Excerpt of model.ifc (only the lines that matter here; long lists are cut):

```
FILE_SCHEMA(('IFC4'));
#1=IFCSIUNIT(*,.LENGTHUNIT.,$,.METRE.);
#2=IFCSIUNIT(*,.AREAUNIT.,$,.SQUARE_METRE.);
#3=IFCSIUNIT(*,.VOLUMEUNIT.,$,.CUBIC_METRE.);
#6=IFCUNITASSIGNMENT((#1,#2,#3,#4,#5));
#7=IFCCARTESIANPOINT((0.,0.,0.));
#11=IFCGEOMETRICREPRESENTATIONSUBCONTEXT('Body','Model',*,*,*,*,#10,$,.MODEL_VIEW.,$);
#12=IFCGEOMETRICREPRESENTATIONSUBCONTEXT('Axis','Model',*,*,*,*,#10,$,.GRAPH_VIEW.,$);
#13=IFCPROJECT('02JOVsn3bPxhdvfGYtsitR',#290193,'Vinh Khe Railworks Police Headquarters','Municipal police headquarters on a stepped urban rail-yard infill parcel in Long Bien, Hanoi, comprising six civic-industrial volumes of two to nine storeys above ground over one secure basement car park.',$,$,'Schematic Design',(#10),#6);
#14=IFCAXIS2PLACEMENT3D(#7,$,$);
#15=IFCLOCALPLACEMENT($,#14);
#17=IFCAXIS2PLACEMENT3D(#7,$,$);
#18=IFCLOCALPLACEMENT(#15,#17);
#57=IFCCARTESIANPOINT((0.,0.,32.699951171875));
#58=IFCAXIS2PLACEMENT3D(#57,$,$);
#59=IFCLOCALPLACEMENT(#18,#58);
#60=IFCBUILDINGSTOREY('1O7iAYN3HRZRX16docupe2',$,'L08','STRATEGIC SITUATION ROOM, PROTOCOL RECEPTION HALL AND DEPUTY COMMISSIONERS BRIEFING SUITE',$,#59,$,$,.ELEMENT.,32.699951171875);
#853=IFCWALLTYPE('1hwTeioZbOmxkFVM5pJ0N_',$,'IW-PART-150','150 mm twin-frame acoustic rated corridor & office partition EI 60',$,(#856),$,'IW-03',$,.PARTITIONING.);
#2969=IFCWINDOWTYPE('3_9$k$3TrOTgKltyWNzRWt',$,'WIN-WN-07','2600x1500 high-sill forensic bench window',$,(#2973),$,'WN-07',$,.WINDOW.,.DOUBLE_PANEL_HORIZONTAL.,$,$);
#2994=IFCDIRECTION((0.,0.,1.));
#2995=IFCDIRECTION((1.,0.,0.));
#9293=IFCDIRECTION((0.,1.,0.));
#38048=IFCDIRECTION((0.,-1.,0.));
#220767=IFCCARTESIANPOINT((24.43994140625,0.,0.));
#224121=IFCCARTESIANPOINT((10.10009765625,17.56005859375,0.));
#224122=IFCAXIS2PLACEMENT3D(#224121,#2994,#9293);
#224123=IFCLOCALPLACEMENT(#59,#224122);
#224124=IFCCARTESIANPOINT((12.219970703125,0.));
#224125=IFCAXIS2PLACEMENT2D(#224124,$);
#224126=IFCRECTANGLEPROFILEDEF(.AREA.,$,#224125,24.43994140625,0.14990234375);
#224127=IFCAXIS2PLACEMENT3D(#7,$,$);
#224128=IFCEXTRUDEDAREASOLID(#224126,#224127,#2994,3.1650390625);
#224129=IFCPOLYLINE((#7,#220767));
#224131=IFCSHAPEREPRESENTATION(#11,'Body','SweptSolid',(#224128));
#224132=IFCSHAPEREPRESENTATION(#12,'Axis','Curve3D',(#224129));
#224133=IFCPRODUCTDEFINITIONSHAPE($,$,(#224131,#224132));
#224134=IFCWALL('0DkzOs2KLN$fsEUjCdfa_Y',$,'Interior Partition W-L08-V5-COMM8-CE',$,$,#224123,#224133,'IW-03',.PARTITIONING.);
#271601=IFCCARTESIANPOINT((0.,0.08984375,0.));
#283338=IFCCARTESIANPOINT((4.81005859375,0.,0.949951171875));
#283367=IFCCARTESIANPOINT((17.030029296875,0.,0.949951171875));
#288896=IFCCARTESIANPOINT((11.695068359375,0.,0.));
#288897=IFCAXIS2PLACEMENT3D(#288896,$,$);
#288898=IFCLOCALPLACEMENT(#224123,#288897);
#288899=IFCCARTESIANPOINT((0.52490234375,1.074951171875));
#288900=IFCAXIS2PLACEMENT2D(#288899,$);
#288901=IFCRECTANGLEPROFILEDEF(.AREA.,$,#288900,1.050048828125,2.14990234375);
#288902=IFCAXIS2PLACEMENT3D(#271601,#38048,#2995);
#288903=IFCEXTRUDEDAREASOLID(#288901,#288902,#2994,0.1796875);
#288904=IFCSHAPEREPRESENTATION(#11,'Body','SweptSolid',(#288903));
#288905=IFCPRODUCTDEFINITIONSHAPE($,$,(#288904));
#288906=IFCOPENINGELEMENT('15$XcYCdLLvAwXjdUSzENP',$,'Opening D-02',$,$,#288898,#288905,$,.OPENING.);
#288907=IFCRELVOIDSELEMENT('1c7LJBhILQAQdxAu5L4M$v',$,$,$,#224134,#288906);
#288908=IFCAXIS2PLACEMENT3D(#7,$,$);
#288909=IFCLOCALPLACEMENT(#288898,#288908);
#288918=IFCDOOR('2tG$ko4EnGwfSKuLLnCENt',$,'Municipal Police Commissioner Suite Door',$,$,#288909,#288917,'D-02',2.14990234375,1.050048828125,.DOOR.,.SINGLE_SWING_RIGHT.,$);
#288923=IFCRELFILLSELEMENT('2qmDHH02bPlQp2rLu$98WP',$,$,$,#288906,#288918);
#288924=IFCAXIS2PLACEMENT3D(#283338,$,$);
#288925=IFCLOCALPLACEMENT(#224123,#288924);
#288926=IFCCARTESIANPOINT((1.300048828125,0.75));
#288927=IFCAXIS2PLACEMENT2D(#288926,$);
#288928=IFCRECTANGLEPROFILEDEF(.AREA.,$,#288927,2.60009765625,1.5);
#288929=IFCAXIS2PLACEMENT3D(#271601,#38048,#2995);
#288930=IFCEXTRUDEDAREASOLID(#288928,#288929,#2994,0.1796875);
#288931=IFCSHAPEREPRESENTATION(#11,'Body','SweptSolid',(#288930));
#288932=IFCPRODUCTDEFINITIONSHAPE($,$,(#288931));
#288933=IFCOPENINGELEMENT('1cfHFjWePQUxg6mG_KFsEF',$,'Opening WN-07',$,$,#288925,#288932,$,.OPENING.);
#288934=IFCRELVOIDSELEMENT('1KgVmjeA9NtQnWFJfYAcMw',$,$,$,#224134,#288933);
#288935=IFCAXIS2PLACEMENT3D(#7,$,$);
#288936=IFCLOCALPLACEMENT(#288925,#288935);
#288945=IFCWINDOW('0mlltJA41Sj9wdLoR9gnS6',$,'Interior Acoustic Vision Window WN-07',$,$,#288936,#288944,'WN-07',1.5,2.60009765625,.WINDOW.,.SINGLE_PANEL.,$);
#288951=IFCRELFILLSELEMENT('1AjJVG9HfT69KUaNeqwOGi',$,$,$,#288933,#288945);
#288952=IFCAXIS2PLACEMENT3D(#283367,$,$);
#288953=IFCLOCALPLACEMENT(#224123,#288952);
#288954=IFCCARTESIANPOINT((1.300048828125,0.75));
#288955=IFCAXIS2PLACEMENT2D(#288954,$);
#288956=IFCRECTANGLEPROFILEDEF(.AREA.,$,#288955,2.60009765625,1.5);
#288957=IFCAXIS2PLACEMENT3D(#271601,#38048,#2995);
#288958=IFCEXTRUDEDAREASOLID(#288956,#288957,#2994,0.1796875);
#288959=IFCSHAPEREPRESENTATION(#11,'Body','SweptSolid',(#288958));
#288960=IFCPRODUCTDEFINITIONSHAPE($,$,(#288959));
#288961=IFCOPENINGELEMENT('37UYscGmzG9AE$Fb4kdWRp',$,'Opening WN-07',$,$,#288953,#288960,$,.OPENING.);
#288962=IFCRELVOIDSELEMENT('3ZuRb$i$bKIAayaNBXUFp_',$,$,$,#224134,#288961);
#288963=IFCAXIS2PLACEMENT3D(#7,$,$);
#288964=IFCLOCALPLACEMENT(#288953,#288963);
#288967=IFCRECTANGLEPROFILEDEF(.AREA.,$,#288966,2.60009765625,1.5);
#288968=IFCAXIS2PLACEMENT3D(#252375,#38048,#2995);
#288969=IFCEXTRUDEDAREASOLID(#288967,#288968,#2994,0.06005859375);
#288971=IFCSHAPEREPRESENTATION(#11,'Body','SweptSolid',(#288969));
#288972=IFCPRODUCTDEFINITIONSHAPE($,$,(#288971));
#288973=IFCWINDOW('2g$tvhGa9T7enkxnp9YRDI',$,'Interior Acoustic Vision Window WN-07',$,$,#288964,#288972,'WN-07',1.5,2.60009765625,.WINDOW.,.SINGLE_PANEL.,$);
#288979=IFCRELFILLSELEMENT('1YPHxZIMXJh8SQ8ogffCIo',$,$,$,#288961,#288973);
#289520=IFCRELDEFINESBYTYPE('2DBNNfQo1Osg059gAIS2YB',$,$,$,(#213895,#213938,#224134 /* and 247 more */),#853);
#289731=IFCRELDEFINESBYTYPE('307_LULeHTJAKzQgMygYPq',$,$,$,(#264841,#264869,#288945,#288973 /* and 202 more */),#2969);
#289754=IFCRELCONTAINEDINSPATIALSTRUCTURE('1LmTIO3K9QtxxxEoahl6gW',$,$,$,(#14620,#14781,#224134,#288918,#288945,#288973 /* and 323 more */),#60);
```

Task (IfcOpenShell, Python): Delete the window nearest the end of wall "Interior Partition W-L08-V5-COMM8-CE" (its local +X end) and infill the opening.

```python
import ifcopenshell
import ifcopenshell.api.feature
import ifcopenshell.api.root
import ifcopenshell.geom
import ifcopenshell.util.shape

model = ifcopenshell.open("model.ifc")
settings = ifcopenshell.geom.settings()


def volume(element):
    """Net volume in cubic metres, openings subtracted."""
    shape = ifcopenshell.geom.create_shape(settings, element)
    return ifcopenshell.util.shape.get_volume(shape.geometry)


window = model.by_guid("2g$tvhGa9T7enkxnp9YRDI")
opening = window.FillsVoids[0].RelatingOpeningElement
wall = opening.VoidsElements[0].RelatingBuildingElement
before = volume(wall)

ifcopenshell.api.root.remove_product(model, product=window)
ifcopenshell.api.feature.remove_feature(model, feature=opening)

after = volume(wall)

print(f"wall volume {before:.3f} -> {after:.3f} m3")

model.write("model_updated.ifc")
```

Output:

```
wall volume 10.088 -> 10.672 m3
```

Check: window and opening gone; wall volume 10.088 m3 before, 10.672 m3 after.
